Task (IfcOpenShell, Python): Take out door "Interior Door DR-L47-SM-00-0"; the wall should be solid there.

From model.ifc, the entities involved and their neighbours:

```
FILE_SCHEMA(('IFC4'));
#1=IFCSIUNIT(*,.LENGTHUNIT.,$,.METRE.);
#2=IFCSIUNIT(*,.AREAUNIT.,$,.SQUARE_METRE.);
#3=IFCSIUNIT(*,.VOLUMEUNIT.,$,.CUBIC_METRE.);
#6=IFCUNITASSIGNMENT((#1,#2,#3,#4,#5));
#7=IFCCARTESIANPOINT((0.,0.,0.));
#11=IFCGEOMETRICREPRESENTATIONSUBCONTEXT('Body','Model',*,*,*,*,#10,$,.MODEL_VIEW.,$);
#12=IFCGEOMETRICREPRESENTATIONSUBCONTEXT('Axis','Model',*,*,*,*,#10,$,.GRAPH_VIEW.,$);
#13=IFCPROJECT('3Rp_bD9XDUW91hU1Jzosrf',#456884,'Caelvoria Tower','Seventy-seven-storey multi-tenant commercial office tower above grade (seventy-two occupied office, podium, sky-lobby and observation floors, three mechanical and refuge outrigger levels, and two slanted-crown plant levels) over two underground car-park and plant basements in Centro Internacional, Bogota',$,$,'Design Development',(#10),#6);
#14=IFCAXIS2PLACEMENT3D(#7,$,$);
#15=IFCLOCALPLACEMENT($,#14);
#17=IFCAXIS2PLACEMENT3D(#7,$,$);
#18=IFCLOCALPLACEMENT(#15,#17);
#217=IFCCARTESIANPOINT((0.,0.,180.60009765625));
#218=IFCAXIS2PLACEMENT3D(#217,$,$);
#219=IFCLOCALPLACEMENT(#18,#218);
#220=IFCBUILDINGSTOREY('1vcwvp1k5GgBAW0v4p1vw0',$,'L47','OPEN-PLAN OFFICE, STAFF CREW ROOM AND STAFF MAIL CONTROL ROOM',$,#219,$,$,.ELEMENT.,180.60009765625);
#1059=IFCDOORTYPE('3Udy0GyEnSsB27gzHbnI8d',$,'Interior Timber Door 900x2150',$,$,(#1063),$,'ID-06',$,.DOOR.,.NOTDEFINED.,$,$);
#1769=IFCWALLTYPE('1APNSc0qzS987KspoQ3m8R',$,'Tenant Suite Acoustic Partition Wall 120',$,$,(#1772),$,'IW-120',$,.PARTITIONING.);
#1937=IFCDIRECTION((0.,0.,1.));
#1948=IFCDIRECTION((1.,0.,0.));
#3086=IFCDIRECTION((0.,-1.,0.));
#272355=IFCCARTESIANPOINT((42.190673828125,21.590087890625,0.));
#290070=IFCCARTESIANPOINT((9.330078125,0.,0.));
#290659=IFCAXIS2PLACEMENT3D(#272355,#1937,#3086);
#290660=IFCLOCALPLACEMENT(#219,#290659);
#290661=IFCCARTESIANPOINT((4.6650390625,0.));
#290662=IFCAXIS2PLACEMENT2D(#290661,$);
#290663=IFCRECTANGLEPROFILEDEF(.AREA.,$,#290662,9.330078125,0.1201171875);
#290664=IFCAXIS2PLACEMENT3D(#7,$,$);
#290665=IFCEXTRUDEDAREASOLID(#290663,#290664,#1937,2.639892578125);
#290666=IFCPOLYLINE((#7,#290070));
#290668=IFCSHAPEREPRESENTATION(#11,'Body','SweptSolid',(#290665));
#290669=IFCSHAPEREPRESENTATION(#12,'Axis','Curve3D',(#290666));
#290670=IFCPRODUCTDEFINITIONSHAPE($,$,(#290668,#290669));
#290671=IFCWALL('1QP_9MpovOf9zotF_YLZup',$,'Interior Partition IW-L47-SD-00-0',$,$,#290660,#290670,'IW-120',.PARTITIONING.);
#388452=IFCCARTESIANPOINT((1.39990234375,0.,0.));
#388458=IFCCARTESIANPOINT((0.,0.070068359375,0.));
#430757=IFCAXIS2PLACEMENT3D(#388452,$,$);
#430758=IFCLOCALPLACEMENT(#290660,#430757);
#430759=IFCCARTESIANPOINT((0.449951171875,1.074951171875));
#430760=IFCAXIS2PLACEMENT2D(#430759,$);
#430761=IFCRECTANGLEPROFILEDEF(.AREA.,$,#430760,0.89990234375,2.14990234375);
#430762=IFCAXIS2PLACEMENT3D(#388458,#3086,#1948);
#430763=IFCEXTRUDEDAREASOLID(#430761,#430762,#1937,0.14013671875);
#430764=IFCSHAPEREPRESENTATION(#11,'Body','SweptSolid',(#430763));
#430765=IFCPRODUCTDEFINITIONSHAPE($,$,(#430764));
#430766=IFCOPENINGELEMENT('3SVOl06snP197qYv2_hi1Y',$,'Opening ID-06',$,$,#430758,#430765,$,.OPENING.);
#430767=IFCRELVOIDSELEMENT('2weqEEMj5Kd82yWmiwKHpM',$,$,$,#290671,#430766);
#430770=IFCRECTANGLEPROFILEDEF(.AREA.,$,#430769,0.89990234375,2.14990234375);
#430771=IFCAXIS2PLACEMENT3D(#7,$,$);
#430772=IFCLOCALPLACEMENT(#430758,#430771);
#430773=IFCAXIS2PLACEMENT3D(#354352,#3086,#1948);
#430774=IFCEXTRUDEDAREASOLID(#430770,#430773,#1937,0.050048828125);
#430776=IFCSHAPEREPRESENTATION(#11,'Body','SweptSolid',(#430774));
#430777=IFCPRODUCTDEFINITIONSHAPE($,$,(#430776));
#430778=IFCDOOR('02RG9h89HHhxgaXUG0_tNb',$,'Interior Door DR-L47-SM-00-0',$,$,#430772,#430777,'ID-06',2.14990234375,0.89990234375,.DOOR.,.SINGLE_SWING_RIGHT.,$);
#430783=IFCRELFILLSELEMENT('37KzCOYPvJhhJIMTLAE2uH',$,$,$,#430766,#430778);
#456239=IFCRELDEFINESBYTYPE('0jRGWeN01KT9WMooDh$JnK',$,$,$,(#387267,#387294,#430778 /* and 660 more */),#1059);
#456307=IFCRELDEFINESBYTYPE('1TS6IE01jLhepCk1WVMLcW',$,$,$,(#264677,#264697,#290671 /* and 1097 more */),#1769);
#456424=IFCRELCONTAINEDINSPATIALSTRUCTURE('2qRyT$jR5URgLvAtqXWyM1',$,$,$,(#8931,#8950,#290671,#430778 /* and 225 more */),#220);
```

```python
import ifcopenshell
import ifcopenshell.api.feature
import ifcopenshell.api.root
import ifcopenshell.geom
import ifcopenshell.util.shape

model = ifcopenshell.open("model.ifc")
settings = ifcopenshell.geom.settings()


def volume(element):
    """Net volume in cubic metres, openings subtracted."""
    shape = ifcopenshell.geom.create_shape(settings, element)
    return ifcopenshell.util.shape.get_volume(shape.geometry)


door = model.by_guid("02RG9h89HHhxgaXUG0_tNb")
opening = door.FillsVoids[0].RelatingOpeningElement
wall = opening.VoidsElements[0].RelatingBuildingElement
before = volume(wall)

ifcopenshell.api.root.remove_product(model, product=door)
ifcopenshell.api.feature.remove_feature(model, feature=opening)

after = volume(wall)

print(f"wall volume {before:.3f} -> {after:.3f} m3")

model.write("model_updated.ifc")
```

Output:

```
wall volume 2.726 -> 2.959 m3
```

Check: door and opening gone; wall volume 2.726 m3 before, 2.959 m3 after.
